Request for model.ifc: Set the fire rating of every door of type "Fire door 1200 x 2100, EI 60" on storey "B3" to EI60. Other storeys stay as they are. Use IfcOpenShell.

First a look at what the model holds.

```python
import ifcopenshell
import ifcopenshell.util.element

model = ifcopenshell.open("model.ifc")
print(model.schema)
storey = next(s for s in model.by_type("IfcBuildingStorey") if s.Name == "B3")
doors = [e for e in ifcopenshell.util.element.get_decomposition(storey) if e.is_a("IfcDoor")]
seen = {}
for e in doors:
    element_type = ifcopenshell.util.element.get_type(e)
    key = (element_type.Name if element_type != e and element_type else None, ifcopenshell.util.element.get_pset(e, "Pset_DoorCommon", "FireRating"))
    seen[key] = seen.get(key, 0) + 1
for (name, value), count in sorted(seen.items(), key=str):
    print(count, "x", name, "|", value)
```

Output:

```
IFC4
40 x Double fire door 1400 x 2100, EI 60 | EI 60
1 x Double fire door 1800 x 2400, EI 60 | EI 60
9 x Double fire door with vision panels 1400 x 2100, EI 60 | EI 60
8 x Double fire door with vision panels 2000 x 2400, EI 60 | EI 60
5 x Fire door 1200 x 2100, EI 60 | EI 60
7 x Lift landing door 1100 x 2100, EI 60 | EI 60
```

```python
import ifcopenshell
import ifcopenshell.api.pset
import ifcopenshell.util.element

model = ifcopenshell.open("model.ifc")

storey = next(s for s in model.by_type("IfcBuildingStorey") if s.Name == "B3")
doors = [e for e in ifcopenshell.util.element.get_decomposition(storey) if e.is_a("IfcDoor")]

count = 0
for e in doors:
    element_type = ifcopenshell.util.element.get_type(e)
    if element_type in (None, e) or element_type.Name != "Fire door 1200 x 2100, EI 60":
        continue
    # add_pset returns the element's existing set when there is one.
    pset = ifcopenshell.api.pset.add_pset(model, product=e, name="Pset_DoorCommon")
    ifcopenshell.api.pset.edit_pset(model, pset=pset, properties={"FireRating": "EI60"})
    count += 1

print(count, "doors updated")

model.write("model-out.ifc")
```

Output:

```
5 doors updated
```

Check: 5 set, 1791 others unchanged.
